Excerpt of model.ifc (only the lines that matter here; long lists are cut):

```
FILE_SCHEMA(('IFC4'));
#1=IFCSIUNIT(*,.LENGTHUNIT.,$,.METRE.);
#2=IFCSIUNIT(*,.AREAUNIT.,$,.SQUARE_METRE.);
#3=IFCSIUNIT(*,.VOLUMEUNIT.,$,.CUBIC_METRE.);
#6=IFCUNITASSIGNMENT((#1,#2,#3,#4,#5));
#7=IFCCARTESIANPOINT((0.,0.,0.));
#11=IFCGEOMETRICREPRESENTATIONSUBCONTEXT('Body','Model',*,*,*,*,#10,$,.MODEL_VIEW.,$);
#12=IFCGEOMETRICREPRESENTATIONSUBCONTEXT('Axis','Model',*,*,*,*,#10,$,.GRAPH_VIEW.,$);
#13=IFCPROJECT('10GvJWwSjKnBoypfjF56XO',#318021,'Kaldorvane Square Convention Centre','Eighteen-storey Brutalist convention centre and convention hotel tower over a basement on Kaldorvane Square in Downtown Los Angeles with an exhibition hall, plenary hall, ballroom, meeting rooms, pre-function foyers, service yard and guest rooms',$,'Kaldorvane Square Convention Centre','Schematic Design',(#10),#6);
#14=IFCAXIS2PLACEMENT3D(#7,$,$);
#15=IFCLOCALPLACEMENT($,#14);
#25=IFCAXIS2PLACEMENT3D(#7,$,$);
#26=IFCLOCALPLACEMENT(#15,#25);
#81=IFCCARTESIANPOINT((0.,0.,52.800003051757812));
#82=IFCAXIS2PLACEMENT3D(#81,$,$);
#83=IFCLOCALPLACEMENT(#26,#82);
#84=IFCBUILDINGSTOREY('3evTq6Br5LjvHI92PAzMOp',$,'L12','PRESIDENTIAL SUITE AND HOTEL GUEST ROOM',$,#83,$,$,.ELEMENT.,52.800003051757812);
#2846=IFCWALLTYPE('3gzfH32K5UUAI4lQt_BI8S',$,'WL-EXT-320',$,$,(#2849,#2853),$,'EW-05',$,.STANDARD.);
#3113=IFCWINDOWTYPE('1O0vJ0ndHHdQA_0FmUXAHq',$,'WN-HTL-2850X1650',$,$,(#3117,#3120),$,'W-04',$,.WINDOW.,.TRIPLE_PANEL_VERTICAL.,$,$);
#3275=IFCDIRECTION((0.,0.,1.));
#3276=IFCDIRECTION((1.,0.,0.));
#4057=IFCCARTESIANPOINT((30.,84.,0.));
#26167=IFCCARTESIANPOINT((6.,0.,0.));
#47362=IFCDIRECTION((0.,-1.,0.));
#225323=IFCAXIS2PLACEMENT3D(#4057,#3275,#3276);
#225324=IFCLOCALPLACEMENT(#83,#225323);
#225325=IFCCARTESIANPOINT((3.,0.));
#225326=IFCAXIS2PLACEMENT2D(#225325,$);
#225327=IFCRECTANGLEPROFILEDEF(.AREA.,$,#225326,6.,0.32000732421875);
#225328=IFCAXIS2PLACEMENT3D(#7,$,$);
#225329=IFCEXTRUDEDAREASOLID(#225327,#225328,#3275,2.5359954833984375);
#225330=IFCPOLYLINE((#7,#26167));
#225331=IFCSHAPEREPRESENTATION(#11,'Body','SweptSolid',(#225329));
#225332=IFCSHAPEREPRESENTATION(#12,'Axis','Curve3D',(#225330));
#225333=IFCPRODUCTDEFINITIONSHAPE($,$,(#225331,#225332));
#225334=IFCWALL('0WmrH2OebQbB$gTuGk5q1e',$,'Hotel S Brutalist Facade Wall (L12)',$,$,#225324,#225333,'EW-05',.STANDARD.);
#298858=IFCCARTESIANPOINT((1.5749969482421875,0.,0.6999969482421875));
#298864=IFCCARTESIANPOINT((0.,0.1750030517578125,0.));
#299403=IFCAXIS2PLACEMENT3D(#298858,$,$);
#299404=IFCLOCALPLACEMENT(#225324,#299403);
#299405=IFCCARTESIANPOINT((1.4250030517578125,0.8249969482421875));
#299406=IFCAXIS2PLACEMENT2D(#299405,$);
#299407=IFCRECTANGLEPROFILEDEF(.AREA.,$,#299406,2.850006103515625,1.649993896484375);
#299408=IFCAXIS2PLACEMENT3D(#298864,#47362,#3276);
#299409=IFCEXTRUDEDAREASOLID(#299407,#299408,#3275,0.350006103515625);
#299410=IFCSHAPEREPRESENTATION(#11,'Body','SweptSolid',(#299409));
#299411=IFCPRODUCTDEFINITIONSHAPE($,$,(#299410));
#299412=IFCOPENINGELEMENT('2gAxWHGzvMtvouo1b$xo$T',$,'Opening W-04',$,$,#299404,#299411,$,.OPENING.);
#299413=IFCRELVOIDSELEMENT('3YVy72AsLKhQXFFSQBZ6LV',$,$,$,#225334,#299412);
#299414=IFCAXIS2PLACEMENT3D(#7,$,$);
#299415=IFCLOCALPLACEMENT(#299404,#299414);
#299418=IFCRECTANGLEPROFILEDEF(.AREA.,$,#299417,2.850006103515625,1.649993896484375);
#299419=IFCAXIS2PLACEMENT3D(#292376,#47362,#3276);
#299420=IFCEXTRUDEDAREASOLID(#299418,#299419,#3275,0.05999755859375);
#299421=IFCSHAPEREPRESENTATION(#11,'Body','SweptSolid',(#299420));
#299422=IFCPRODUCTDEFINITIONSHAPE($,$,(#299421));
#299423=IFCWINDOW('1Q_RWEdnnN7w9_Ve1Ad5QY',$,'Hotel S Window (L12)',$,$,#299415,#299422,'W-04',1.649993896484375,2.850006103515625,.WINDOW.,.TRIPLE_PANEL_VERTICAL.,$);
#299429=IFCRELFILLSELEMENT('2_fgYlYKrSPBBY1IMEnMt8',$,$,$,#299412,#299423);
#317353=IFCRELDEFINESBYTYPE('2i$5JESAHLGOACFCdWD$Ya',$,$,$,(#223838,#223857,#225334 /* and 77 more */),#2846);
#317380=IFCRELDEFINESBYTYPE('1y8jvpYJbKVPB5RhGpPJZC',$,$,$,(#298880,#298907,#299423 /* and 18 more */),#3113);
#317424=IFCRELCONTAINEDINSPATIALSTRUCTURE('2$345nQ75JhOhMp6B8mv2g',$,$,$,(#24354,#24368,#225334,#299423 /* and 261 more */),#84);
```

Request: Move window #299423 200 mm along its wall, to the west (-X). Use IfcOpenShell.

```python
import ifcopenshell
import ifcopenshell.api.geometry
import ifcopenshell.util.placement

model = ifcopenshell.open("model.ifc")

window = model.by_id(299423)
opening = window.FillsVoids[0].RelatingOpeningElement
wall = opening.VoidsElements[0].RelatingBuildingElement

wall_matrix = ifcopenshell.util.placement.get_local_placement(wall.ObjectPlacement)
shift = wall_matrix[:3, 0] * -0.2
before = ifcopenshell.util.placement.get_local_placement(window.ObjectPlacement)[:3, 3].copy()

# The window is placed relative to its opening, so it follows when the opening moves.
matrix = ifcopenshell.util.placement.get_local_placement(opening.ObjectPlacement)
matrix[:3, 3] += shift
ifcopenshell.api.geometry.edit_object_placement(
    model, product=opening, matrix=matrix, is_si=False, should_transform_children=True
)

after = ifcopenshell.util.placement.get_local_placement(window.ObjectPlacement)[:3, 3]
print("window moved by", (after - before).round(3) + 0.0)

model.write("model_edited.ifc")
```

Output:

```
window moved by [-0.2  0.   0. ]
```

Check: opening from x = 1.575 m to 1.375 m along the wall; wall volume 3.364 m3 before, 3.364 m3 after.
